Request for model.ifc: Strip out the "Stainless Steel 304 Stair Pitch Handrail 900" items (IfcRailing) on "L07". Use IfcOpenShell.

First a look at what the model holds.

```python
import ifcopenshell
import ifcopenshell.util.element

model = ifcopenshell.open("model.ifc")
print(model.schema)
storey = next(s for s in model.by_type("IfcBuildingStorey") if s.Name == "L07")
railings = [e for e in ifcopenshell.util.element.get_decomposition(storey) if e.is_a("IfcRailing")]
seen = {}
for e in railings:
    element_type = ifcopenshell.util.element.get_type(e)
    name = element_type.Name if element_type not in (None, e) else None
    seen[name] = seen.get(name, 0) + 1
for name, count in sorted(seen.items(), key=str):
    print(count, "x", name)
```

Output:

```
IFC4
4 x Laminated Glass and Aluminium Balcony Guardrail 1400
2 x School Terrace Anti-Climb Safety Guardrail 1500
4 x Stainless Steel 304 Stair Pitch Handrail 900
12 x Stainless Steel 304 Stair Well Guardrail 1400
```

```python
import ifcopenshell
import ifcopenshell.api.root
import ifcopenshell.util.element

model = ifcopenshell.open("model.ifc")

storey = next(s for s in model.by_type("IfcBuildingStorey") if s.Name == "L07")
railings = [e for e in ifcopenshell.util.element.get_decomposition(storey) if e.is_a("IfcRailing")]
targets = [e for e in railings if (t := ifcopenshell.util.element.get_type(e)) not in (None, e) and t.Name == "Stainless Steel 304 Stair Pitch Handrail 900"]

for e in targets:
    ifcopenshell.api.root.remove_product(model, product=e)
print(len(targets), "removed")

model.write("model_updated.ifc")
```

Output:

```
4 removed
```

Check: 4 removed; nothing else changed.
